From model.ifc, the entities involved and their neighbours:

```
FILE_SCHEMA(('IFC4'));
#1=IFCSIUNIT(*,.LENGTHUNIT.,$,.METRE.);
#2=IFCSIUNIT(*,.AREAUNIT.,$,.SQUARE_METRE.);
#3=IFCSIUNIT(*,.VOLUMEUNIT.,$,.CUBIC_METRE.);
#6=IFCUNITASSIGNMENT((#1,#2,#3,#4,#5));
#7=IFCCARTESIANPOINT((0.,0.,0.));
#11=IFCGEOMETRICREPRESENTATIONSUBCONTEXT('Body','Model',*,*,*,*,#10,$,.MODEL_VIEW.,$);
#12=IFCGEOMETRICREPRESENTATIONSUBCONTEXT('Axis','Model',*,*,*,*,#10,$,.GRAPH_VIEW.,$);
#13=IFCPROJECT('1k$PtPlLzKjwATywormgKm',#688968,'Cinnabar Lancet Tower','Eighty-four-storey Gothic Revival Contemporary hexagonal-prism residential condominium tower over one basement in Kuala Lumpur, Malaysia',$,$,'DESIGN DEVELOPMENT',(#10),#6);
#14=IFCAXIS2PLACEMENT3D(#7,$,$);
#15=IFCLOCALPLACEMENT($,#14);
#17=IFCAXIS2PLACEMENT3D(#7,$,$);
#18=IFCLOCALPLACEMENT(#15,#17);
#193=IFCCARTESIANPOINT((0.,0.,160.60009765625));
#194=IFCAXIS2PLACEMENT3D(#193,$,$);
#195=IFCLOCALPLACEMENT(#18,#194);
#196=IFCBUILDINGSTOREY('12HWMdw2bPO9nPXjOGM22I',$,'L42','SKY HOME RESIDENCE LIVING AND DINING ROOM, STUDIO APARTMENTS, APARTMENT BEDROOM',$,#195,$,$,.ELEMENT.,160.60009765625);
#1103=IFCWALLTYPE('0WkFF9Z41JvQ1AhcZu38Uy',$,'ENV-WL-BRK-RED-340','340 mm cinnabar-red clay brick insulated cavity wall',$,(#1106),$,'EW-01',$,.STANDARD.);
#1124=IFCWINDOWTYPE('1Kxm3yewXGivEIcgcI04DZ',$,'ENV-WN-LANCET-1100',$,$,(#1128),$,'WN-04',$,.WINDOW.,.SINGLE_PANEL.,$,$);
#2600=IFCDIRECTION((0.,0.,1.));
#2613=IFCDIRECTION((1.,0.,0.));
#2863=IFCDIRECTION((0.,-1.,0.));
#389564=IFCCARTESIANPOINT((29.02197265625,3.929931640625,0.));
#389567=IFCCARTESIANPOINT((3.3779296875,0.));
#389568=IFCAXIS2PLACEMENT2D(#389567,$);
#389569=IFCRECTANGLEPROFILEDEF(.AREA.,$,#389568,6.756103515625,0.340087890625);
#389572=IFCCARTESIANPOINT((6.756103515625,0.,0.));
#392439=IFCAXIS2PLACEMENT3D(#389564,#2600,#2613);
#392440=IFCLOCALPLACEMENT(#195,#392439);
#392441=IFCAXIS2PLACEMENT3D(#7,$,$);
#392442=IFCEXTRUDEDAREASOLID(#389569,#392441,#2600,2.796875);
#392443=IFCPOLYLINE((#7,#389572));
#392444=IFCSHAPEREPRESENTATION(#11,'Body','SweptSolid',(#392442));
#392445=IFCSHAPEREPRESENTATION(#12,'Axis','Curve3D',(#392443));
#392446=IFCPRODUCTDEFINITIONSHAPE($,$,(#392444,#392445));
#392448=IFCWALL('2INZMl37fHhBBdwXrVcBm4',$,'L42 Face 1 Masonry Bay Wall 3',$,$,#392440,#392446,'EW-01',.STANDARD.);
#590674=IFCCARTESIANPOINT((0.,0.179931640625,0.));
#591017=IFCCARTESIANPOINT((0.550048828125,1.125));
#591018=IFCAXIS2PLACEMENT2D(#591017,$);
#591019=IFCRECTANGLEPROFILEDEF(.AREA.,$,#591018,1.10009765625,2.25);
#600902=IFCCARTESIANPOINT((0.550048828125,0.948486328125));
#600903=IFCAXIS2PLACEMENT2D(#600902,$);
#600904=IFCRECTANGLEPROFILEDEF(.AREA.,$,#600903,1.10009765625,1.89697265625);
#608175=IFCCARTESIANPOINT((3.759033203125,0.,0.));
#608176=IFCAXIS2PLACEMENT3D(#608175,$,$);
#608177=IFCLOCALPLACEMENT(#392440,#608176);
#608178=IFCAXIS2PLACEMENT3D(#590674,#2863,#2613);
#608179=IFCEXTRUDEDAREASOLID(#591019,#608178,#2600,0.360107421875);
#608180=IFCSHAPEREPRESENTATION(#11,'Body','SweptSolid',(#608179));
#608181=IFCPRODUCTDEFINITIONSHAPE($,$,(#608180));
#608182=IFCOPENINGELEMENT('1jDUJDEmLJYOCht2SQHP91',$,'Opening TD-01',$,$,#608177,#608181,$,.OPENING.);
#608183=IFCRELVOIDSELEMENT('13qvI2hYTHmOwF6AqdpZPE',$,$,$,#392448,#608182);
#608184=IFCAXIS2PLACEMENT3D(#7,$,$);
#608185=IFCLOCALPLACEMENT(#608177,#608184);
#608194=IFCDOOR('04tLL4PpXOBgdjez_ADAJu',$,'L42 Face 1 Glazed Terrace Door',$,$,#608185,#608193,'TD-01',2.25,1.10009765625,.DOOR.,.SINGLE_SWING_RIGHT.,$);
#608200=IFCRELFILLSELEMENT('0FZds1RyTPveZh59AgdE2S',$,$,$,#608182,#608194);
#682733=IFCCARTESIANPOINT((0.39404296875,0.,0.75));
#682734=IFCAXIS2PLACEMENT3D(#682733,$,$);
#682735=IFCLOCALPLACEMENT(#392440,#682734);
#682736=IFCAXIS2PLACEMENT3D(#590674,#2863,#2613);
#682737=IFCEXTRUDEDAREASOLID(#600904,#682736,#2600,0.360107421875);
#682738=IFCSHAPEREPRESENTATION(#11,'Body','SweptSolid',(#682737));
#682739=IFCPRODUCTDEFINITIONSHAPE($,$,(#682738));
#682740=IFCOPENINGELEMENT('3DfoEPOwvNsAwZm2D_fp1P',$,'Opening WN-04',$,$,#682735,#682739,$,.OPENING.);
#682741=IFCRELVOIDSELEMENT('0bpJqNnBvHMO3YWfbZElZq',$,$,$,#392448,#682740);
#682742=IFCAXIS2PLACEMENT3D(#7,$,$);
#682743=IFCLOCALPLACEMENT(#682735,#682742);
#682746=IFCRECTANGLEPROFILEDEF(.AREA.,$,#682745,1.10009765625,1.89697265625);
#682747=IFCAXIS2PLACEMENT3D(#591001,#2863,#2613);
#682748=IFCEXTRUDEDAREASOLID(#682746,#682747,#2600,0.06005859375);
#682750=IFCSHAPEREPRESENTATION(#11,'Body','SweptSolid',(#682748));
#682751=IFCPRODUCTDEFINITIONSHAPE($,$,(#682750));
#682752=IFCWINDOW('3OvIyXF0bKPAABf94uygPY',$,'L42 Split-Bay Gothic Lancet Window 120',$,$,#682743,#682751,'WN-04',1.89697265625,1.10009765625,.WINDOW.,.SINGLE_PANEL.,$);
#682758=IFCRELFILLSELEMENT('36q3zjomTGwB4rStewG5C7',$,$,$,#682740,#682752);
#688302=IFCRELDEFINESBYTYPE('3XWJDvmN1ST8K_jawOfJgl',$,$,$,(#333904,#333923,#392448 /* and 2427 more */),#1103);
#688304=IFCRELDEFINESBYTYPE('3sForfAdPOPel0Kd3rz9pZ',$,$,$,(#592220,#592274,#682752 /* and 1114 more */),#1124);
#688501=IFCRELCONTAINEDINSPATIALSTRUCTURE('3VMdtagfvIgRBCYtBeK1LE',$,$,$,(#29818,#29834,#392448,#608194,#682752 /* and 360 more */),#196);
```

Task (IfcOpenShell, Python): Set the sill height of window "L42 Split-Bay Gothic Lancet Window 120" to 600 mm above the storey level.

```python
import numpy as np
import ifcopenshell
import ifcopenshell.api.geometry
import ifcopenshell.geom
import ifcopenshell.util.element
import ifcopenshell.util.placement
import ifcopenshell.util.shape
import ifcopenshell.util.unit

model = ifcopenshell.open("model.ifc")
unit_scale = ifcopenshell.util.unit.calculate_unit_scale(model)

window = model.by_id(682752)
opening = window.FillsVoids[0].RelatingOpeningElement
storey = ifcopenshell.util.element.get_container(window, ifc_class="IfcBuildingStorey")
level = ifcopenshell.util.placement.get_local_placement(storey.ObjectPlacement)[2, 3]

# The opening's origin need not be at the sill, so measure its lowest point.
shape = ifcopenshell.geom.create_shape(ifcopenshell.geom.settings(), opening)
bottom = ifcopenshell.util.shape.get_shape_bottom_elevation(shape, shape.geometry) / unit_scale
dz = level + 0.6 - bottom

shift = np.array([0.0, 0.0, dz])
# The window is placed relative to its opening, so it follows when the opening moves.
matrix = ifcopenshell.util.placement.get_local_placement(opening.ObjectPlacement)
matrix[:3, 3] += shift
ifcopenshell.api.geometry.edit_object_placement(
    model, product=opening, matrix=matrix, is_si=False, should_transform_children=True
)

print(f"moved by {dz * unit_scale:+.3f} m")

model.write("model_rev.ifc")
```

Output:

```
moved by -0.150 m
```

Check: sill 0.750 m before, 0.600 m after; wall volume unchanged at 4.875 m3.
